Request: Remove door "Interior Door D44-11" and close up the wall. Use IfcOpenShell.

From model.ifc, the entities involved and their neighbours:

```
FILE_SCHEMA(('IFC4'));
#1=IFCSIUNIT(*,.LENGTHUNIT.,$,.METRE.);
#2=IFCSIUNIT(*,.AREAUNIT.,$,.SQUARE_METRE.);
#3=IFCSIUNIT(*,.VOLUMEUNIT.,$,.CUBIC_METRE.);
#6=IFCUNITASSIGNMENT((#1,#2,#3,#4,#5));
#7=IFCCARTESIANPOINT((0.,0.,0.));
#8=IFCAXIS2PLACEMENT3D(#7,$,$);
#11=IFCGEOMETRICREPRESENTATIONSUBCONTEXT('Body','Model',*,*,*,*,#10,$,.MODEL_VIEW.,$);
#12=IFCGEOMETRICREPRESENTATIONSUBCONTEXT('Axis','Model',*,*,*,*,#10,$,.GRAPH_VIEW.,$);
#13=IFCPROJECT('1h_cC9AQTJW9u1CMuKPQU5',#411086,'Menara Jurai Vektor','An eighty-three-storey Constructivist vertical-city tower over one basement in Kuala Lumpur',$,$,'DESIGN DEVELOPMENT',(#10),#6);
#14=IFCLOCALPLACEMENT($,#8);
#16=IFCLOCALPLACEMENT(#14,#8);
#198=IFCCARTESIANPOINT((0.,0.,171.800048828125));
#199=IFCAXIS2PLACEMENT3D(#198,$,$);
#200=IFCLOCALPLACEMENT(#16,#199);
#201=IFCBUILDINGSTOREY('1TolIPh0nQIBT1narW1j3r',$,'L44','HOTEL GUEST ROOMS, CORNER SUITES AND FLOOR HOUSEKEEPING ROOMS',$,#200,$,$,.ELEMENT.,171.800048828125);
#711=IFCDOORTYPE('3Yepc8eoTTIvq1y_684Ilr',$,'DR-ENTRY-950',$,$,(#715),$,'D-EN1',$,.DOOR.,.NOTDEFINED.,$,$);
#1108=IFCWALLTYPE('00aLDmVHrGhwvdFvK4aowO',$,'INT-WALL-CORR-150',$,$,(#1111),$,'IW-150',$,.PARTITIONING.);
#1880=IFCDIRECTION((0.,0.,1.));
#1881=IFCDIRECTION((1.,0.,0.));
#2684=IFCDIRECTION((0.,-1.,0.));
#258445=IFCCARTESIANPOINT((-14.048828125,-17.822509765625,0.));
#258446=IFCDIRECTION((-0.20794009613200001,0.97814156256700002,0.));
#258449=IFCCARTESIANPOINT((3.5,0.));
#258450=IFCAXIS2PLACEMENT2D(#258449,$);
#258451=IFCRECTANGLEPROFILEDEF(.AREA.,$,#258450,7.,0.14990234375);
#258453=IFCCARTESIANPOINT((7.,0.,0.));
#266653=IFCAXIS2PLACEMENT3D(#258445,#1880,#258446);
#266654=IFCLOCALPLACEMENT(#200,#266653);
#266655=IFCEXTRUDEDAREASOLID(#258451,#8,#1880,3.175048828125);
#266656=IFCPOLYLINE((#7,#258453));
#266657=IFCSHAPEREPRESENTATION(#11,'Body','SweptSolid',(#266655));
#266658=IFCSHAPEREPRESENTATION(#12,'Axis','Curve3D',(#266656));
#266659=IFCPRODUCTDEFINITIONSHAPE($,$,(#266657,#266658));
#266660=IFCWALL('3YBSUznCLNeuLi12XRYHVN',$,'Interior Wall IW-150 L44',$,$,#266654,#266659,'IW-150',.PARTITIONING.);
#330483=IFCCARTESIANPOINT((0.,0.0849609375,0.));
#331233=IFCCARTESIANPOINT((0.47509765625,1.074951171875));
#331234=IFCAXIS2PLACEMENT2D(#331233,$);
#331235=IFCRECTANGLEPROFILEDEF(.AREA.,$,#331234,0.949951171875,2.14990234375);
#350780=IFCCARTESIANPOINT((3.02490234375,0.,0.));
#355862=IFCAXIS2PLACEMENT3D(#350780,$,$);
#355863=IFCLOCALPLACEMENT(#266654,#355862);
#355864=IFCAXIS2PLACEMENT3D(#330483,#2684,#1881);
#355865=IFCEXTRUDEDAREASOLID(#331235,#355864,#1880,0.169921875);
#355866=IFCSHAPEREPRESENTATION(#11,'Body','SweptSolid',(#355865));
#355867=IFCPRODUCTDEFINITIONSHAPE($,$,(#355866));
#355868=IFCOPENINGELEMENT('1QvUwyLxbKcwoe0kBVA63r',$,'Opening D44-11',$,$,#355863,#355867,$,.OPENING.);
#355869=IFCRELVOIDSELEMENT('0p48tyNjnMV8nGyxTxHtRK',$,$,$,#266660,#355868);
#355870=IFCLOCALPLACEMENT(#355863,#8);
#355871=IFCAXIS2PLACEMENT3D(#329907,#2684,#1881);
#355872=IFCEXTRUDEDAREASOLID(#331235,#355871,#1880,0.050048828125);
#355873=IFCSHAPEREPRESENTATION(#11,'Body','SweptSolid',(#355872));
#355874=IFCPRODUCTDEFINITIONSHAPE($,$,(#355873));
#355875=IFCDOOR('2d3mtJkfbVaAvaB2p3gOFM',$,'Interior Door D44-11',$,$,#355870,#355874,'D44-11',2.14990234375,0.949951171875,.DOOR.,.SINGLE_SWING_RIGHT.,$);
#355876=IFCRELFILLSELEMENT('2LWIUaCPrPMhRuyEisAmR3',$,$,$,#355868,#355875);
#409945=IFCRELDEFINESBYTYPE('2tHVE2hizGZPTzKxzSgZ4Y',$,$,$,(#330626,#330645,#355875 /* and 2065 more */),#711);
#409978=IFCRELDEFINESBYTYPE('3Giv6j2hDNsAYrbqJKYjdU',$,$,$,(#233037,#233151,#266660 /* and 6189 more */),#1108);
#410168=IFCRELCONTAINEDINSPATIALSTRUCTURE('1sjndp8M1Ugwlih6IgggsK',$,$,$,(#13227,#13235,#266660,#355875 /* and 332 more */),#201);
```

```python
import ifcopenshell
import ifcopenshell.api.feature
import ifcopenshell.api.root
import ifcopenshell.geom
import ifcopenshell.util.shape

model = ifcopenshell.open("model.ifc")
settings = ifcopenshell.geom.settings()


def volume(element):
    """Net volume in cubic metres, openings subtracted."""
    shape = ifcopenshell.geom.create_shape(settings, element)
    return ifcopenshell.util.shape.get_volume(shape.geometry)


door = model.by_guid("2d3mtJkfbVaAvaB2p3gOFM")
opening = door.FillsVoids[0].RelatingOpeningElement
wall = opening.VoidsElements[0].RelatingBuildingElement
before = volume(wall)

ifcopenshell.api.root.remove_product(model, product=door)
ifcopenshell.api.feature.remove_feature(model, feature=opening)

after = volume(wall)

print(f"wall volume {before:.3f} -> {after:.3f} m3")

model.write("model_v2.ifc")
```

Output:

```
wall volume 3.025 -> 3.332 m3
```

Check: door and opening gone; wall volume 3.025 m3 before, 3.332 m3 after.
